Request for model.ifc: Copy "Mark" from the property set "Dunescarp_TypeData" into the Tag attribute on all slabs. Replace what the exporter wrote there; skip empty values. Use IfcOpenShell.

First a look at what the model holds.

```python
import ifcopenshell
import ifcopenshell.util.element

model = ifcopenshell.open("model.ifc")
print(model.schema)
slabs = model.by_type("IfcSlab")
print(len(slabs), "slabs")
for e in slabs[:8]:
    source = ifcopenshell.util.element.get_pset(e, "Dunescarp_TypeData", "Mark")
    target = e.Tag
    print(e.id(), repr(source), repr(target), sep=" | ")
```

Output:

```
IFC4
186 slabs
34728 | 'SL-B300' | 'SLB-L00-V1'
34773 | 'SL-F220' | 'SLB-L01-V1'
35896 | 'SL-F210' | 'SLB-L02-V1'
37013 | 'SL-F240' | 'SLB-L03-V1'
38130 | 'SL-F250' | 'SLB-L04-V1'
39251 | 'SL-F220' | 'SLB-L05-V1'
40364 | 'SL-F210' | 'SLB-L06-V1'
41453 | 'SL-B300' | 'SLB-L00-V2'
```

```python
import ifcopenshell
import ifcopenshell.util.element

model = ifcopenshell.open("model.ifc")

count = 0
for e in model.by_type("IfcSlab"):
    value = ifcopenshell.util.element.get_pset(e, "Dunescarp_TypeData", "Mark")
    current = e.Tag
    if not value or not value.strip() or current == value:
        continue
    e.Tag = value
    count += 1

print(count, "slabs updated")

model.write("model_rev.ifc")
```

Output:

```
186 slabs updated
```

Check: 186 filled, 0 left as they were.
